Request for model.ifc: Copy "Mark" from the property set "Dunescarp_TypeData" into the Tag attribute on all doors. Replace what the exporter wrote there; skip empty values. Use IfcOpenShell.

First a look at what the model holds.

```python
import ifcopenshell
import ifcopenshell.util.element

model = ifcopenshell.open("model.ifc")
print(model.schema)
doors = model.by_type("IfcDoor")
print(len(doors), "doors")
for e in doors[:8]:
    source = ifcopenshell.util.element.get_pset(e, "Dunescarp_TypeData", "Mark")
    target = e.Tag
    print(e.id(), repr(source), repr(target), sep=" | ")
```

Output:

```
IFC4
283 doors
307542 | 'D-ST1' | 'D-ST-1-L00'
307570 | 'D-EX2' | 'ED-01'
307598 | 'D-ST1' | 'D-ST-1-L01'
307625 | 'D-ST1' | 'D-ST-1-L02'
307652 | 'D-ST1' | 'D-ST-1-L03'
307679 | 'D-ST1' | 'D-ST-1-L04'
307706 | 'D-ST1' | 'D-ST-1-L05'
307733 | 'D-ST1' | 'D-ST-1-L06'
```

```python
import ifcopenshell
import ifcopenshell.util.element

model = ifcopenshell.open("model.ifc")

count = 0
for e in model.by_type("IfcDoor"):
    value = ifcopenshell.util.element.get_pset(e, "Dunescarp_TypeData", "Mark")
    current = e.Tag
    if not value or not value.strip() or current == value:
        continue
    e.Tag = value
    count += 1

print(count, "doors updated")

model.write("model_edited.ifc")
```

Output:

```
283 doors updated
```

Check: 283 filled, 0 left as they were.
